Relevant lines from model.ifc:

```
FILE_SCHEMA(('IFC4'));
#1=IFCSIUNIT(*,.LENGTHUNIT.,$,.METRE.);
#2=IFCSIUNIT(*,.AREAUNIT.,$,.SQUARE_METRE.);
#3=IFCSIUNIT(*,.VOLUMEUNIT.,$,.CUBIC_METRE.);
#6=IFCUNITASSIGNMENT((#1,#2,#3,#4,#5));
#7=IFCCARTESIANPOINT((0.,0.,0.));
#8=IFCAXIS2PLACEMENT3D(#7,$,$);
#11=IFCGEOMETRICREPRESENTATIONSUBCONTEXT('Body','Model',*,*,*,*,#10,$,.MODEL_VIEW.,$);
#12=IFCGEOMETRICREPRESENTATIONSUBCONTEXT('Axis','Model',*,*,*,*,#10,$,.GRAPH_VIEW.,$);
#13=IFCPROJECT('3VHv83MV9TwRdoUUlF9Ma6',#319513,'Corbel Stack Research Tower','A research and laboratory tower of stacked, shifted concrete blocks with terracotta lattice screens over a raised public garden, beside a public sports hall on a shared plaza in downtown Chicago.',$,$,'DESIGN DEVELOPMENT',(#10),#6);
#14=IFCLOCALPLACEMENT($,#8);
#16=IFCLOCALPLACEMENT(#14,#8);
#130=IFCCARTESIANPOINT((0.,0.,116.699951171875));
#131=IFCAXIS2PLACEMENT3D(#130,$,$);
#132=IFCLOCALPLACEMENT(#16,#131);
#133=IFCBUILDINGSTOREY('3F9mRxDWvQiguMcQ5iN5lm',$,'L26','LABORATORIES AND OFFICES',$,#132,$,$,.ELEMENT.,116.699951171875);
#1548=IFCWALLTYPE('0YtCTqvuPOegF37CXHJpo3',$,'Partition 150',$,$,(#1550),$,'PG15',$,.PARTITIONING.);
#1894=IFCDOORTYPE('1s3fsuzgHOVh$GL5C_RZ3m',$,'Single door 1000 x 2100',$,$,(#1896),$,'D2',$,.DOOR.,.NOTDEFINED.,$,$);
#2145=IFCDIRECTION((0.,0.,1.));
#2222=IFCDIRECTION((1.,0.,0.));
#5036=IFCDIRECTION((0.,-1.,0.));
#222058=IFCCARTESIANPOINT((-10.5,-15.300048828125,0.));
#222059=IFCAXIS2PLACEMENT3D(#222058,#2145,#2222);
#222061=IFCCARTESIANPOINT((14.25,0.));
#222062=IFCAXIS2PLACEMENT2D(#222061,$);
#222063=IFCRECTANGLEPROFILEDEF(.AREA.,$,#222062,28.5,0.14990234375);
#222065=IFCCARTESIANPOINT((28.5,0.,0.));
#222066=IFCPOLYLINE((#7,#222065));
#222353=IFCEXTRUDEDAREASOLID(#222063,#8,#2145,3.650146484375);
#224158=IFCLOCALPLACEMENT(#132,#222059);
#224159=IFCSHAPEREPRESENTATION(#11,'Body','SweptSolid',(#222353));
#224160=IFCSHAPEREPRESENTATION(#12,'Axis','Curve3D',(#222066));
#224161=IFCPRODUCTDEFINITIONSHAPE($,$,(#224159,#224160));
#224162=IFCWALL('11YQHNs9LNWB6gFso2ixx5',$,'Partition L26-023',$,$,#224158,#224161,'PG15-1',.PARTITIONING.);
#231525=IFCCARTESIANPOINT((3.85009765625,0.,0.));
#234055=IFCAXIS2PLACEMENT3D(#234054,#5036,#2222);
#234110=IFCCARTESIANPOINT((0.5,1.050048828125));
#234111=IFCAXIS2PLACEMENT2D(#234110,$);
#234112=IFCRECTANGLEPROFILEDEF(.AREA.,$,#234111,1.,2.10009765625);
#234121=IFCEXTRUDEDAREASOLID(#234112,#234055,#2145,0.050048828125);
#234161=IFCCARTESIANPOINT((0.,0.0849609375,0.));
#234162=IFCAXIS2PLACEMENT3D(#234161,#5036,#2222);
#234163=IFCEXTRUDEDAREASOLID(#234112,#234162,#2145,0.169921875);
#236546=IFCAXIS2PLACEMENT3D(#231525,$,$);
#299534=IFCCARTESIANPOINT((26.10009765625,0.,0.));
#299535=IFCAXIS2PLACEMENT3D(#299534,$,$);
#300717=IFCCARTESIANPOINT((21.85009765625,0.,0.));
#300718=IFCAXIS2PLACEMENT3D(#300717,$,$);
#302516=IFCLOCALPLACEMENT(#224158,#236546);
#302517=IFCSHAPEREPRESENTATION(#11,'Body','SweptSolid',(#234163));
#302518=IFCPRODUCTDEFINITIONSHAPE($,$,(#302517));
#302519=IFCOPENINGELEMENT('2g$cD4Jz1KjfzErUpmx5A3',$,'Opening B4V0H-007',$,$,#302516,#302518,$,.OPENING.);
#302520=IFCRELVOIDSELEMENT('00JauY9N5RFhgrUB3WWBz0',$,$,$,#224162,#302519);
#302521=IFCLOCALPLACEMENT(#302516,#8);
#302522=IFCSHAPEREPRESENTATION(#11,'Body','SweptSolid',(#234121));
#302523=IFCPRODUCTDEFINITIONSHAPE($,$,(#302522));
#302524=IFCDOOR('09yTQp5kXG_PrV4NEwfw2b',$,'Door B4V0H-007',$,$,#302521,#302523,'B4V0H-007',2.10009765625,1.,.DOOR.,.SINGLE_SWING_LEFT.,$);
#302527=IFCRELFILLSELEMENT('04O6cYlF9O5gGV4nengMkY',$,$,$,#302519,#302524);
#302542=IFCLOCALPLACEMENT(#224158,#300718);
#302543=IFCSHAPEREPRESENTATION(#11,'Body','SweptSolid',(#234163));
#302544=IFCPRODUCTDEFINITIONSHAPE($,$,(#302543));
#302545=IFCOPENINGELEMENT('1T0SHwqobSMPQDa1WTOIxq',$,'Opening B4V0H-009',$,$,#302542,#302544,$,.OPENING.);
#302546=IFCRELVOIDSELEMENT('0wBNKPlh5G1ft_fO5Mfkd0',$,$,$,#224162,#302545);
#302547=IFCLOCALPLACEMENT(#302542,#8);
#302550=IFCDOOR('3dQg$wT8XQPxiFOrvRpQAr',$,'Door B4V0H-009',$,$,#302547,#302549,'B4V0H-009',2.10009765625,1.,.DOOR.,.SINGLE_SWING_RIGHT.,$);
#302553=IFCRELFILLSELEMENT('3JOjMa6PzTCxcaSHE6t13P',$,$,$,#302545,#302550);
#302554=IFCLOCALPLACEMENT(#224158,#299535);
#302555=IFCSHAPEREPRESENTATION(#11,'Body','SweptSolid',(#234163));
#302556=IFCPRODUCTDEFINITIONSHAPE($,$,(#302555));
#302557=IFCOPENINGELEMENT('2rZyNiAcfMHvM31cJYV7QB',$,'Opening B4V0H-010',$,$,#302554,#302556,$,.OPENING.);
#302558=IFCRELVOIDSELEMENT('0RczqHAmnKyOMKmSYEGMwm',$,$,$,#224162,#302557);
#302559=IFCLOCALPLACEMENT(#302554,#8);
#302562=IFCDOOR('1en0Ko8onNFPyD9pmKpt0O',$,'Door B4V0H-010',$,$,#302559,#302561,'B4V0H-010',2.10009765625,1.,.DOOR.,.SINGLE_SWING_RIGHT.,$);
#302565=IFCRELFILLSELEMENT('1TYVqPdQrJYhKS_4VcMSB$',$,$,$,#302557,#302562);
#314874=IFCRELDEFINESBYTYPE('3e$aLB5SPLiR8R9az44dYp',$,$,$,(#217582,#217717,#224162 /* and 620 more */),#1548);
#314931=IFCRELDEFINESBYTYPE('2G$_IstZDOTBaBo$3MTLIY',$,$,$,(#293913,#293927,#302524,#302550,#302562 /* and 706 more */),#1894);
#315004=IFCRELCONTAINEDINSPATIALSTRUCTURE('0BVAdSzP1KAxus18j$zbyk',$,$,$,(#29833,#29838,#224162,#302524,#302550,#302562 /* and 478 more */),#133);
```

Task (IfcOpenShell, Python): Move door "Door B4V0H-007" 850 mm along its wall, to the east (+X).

```python
import ifcopenshell
import ifcopenshell.api.geometry
import ifcopenshell.util.placement

model = ifcopenshell.open("model.ifc")

door = model.by_id(302524)
opening = door.FillsVoids[0].RelatingOpeningElement
wall = opening.VoidsElements[0].RelatingBuildingElement

wall_matrix = ifcopenshell.util.placement.get_local_placement(wall.ObjectPlacement)
shift = wall_matrix[:3, 0] * 0.85
before = ifcopenshell.util.placement.get_local_placement(door.ObjectPlacement)[:3, 3].copy()

# The door is placed relative to its opening, so it follows when the opening moves.
matrix = ifcopenshell.util.placement.get_local_placement(opening.ObjectPlacement)
matrix[:3, 3] += shift
ifcopenshell.api.geometry.edit_object_placement(
    model, product=opening, matrix=matrix, is_si=False, should_transform_children=True
)

after = ifcopenshell.util.placement.get_local_placement(door.ObjectPlacement)[:3, 3]
print("door moved by", (after - before).round(3) + 0.0)

model.write("model-out.ifc")
```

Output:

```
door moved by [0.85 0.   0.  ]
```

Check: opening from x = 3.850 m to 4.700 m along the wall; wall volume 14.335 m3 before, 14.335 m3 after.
